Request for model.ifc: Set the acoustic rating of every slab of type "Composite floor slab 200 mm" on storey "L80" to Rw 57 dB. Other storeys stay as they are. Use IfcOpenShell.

First a look at what the model holds.

```python
import ifcopenshell
import ifcopenshell.util.element

model = ifcopenshell.open("model.ifc")
print(model.schema)
storey = next(s for s in model.by_type("IfcBuildingStorey") if s.Name == "L80")
slabs = [e for e in ifcopenshell.util.element.get_decomposition(storey) if e.is_a("IfcSlab")]
seen = {}
for e in slabs:
    element_type = ifcopenshell.util.element.get_type(e)
    key = (element_type.Name if element_type != e and element_type else None, ifcopenshell.util.element.get_pset(e, "Pset_SlabCommon", "AcousticRating"))
    seen[key] = seen.get(key, 0) + 1
for (name, value), count in sorted(seen.items(), key=str):
    print(count, "x", name, "|", value)
```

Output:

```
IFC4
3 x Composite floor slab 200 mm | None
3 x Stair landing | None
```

```python
import ifcopenshell
import ifcopenshell.api.pset
import ifcopenshell.util.element

model = ifcopenshell.open("model.ifc")

storey = next(s for s in model.by_type("IfcBuildingStorey") if s.Name == "L80")
slabs = [e for e in ifcopenshell.util.element.get_decomposition(storey) if e.is_a("IfcSlab")]

count = 0
for e in slabs:
    element_type = ifcopenshell.util.element.get_type(e)
    if element_type in (None, e) or element_type.Name != "Composite floor slab 200 mm":
        continue
    found = ifcopenshell.util.element.get_pset(e, "Pset_SlabCommon", should_inherit=False)
    if found:
        pset = model.by_id(found["id"])
        if len(ifcopenshell.util.element.get_elements_by_pset(pset)) > 1:
            pset = ifcopenshell.api.pset.unshare_pset(model, products=[e], pset=pset)[0]
    else:
        pset = ifcopenshell.api.pset.add_pset(model, product=e, name="Pset_SlabCommon")
    ifcopenshell.api.pset.edit_pset(model, pset=pset, properties={"AcousticRating": "Rw 57 dB"})
    count += 1

print(count, "slabs updated")

model.write("model_rev.ifc")
```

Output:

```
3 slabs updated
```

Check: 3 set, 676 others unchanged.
